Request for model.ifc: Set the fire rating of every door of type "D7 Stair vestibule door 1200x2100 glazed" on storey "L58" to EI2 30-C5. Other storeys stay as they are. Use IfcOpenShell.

First a look at what the model holds.

```python
import ifcopenshell
import ifcopenshell.util.element

model = ifcopenshell.open("model.ifc")
print(model.schema)
storey = next(s for s in model.by_type("IfcBuildingStorey") if s.Name == "L58")
doors = [e for e in ifcopenshell.util.element.get_decomposition(storey) if e.is_a("IfcDoor")]
seen = {}
for e in doors:
    element_type = ifcopenshell.util.element.get_type(e)
    key = (element_type.Name if element_type != e and element_type else None, ifcopenshell.util.element.get_pset(e, "Pset_DoorCommon", "FireRating"))
    seen[key] = seen.get(key, 0) + 1
for (name, value), count in sorted(seen.items(), key=str):
    print(count, "x", name, "|", value)
```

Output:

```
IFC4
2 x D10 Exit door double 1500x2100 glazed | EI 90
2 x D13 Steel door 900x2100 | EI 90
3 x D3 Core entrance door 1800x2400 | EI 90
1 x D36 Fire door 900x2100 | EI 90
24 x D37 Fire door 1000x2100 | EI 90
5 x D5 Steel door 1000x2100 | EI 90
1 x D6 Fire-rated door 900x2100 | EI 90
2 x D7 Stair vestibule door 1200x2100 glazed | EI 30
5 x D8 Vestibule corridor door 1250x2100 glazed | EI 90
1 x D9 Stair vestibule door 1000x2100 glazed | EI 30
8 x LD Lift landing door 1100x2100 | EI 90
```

```python
import ifcopenshell
import ifcopenshell.api.pset
import ifcopenshell.util.element

model = ifcopenshell.open("model.ifc")

storey = next(s for s in model.by_type("IfcBuildingStorey") if s.Name == "L58")
doors = [e for e in ifcopenshell.util.element.get_decomposition(storey) if e.is_a("IfcDoor")]

count = 0
for e in doors:
    element_type = ifcopenshell.util.element.get_type(e)
    if element_type in (None, e) or element_type.Name != "D7 Stair vestibule door 1200x2100 glazed":
        continue
    found = ifcopenshell.util.element.get_pset(e, "Pset_DoorCommon", should_inherit=False)
    if found:
        pset = model.by_id(found["id"])
        if len(ifcopenshell.util.element.get_elements_by_pset(pset)) > 1:
            pset = ifcopenshell.api.pset.unshare_pset(model, products=[e], pset=pset)[0]
    else:
        pset = ifcopenshell.api.pset.add_pset(model, product=e, name="Pset_DoorCommon")
    ifcopenshell.api.pset.edit_pset(model, pset=pset, properties={"FireRating": "EI2 30-C5"})
    count += 1

print(count, "doors updated")

model.write("model_updated.ifc")
```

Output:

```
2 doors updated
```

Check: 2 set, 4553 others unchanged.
